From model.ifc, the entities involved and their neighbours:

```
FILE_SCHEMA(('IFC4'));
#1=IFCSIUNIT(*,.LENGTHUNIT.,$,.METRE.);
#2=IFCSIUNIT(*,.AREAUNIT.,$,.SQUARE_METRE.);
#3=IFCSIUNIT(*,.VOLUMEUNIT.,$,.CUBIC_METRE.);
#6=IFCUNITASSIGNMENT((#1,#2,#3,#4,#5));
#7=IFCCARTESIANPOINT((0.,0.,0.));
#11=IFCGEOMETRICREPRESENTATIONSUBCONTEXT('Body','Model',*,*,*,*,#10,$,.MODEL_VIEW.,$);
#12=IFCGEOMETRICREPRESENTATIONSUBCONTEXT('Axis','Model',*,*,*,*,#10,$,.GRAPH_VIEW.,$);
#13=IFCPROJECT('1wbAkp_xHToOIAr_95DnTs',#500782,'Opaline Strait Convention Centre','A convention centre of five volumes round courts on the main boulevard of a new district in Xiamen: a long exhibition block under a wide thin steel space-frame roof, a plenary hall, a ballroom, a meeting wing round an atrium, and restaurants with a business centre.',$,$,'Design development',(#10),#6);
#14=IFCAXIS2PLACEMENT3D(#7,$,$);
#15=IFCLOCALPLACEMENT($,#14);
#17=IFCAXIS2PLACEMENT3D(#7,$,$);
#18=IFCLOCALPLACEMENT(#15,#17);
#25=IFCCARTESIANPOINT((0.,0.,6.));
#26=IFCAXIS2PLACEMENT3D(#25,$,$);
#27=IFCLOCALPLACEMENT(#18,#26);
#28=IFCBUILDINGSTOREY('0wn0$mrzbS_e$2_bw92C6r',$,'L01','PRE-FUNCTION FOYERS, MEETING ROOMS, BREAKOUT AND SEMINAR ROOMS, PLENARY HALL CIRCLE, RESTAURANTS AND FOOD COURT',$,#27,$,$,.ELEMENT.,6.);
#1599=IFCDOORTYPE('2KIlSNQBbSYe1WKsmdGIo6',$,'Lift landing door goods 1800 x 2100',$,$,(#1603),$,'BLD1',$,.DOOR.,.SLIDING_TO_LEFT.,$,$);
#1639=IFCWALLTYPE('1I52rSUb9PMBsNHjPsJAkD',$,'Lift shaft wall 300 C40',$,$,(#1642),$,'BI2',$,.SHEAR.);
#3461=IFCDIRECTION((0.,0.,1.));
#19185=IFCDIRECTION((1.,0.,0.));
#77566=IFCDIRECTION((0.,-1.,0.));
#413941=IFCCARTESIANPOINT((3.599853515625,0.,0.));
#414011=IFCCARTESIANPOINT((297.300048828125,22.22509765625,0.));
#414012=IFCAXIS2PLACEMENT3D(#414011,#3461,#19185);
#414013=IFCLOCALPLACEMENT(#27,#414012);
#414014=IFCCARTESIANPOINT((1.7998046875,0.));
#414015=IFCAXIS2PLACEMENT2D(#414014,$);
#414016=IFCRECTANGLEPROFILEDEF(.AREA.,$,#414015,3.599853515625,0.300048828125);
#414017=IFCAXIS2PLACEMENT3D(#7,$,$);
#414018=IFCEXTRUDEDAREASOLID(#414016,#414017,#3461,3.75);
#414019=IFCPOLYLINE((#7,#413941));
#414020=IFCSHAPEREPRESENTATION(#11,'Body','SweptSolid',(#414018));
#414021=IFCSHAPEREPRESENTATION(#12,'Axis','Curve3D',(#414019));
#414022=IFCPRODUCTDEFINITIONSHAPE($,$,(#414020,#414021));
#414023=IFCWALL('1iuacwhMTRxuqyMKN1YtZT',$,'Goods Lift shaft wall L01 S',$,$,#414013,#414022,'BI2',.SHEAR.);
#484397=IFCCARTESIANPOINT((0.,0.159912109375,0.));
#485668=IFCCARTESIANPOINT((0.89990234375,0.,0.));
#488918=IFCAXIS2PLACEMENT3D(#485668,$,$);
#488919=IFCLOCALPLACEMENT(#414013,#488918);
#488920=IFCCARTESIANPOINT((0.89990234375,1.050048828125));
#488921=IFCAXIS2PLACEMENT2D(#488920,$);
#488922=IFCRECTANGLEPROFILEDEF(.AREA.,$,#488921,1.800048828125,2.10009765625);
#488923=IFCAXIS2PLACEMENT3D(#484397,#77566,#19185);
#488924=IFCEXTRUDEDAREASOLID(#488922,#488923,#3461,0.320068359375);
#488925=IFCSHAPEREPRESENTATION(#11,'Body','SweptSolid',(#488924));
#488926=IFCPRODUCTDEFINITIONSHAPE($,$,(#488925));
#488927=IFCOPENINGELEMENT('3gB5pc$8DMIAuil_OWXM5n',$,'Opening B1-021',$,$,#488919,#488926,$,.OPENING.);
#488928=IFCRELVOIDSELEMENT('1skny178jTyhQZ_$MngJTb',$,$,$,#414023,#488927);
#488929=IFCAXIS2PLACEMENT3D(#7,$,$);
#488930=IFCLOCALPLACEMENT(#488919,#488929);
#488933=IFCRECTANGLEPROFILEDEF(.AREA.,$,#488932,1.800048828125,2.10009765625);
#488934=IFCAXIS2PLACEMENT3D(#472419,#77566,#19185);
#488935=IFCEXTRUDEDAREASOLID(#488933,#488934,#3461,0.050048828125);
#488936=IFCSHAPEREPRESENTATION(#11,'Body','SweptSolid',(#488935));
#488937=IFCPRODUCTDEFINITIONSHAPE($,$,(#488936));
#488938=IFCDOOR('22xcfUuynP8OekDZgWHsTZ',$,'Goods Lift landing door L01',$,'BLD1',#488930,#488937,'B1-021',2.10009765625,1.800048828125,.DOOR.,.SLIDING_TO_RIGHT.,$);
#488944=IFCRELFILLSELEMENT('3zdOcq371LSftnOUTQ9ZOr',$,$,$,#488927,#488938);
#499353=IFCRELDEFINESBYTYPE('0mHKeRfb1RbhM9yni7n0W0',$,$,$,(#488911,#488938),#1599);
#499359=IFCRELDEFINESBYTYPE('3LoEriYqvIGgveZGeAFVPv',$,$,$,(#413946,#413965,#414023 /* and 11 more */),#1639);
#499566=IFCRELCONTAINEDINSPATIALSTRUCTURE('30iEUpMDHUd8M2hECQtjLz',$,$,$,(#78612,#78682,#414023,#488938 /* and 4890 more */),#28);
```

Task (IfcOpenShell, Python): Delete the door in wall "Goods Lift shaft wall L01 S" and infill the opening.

```python
import ifcopenshell
import ifcopenshell.api.feature
import ifcopenshell.api.root
import ifcopenshell.geom
import ifcopenshell.util.shape

model = ifcopenshell.open("model.ifc")
settings = ifcopenshell.geom.settings()


def volume(element):
    """Net volume in cubic metres, openings subtracted."""
    shape = ifcopenshell.geom.create_shape(settings, element)
    return ifcopenshell.util.shape.get_volume(shape.geometry)


door = model.by_guid("22xcfUuynP8OekDZgWHsTZ")
opening = door.FillsVoids[0].RelatingOpeningElement
wall = opening.VoidsElements[0].RelatingBuildingElement
before = volume(wall)

ifcopenshell.api.root.remove_product(model, product=door)
ifcopenshell.api.feature.remove_feature(model, feature=opening)

after = volume(wall)

print(f"wall volume {before:.3f} -> {after:.3f} m3")

model.write("model-out.ifc")
```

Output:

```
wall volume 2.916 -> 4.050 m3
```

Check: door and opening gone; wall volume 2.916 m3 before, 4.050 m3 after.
